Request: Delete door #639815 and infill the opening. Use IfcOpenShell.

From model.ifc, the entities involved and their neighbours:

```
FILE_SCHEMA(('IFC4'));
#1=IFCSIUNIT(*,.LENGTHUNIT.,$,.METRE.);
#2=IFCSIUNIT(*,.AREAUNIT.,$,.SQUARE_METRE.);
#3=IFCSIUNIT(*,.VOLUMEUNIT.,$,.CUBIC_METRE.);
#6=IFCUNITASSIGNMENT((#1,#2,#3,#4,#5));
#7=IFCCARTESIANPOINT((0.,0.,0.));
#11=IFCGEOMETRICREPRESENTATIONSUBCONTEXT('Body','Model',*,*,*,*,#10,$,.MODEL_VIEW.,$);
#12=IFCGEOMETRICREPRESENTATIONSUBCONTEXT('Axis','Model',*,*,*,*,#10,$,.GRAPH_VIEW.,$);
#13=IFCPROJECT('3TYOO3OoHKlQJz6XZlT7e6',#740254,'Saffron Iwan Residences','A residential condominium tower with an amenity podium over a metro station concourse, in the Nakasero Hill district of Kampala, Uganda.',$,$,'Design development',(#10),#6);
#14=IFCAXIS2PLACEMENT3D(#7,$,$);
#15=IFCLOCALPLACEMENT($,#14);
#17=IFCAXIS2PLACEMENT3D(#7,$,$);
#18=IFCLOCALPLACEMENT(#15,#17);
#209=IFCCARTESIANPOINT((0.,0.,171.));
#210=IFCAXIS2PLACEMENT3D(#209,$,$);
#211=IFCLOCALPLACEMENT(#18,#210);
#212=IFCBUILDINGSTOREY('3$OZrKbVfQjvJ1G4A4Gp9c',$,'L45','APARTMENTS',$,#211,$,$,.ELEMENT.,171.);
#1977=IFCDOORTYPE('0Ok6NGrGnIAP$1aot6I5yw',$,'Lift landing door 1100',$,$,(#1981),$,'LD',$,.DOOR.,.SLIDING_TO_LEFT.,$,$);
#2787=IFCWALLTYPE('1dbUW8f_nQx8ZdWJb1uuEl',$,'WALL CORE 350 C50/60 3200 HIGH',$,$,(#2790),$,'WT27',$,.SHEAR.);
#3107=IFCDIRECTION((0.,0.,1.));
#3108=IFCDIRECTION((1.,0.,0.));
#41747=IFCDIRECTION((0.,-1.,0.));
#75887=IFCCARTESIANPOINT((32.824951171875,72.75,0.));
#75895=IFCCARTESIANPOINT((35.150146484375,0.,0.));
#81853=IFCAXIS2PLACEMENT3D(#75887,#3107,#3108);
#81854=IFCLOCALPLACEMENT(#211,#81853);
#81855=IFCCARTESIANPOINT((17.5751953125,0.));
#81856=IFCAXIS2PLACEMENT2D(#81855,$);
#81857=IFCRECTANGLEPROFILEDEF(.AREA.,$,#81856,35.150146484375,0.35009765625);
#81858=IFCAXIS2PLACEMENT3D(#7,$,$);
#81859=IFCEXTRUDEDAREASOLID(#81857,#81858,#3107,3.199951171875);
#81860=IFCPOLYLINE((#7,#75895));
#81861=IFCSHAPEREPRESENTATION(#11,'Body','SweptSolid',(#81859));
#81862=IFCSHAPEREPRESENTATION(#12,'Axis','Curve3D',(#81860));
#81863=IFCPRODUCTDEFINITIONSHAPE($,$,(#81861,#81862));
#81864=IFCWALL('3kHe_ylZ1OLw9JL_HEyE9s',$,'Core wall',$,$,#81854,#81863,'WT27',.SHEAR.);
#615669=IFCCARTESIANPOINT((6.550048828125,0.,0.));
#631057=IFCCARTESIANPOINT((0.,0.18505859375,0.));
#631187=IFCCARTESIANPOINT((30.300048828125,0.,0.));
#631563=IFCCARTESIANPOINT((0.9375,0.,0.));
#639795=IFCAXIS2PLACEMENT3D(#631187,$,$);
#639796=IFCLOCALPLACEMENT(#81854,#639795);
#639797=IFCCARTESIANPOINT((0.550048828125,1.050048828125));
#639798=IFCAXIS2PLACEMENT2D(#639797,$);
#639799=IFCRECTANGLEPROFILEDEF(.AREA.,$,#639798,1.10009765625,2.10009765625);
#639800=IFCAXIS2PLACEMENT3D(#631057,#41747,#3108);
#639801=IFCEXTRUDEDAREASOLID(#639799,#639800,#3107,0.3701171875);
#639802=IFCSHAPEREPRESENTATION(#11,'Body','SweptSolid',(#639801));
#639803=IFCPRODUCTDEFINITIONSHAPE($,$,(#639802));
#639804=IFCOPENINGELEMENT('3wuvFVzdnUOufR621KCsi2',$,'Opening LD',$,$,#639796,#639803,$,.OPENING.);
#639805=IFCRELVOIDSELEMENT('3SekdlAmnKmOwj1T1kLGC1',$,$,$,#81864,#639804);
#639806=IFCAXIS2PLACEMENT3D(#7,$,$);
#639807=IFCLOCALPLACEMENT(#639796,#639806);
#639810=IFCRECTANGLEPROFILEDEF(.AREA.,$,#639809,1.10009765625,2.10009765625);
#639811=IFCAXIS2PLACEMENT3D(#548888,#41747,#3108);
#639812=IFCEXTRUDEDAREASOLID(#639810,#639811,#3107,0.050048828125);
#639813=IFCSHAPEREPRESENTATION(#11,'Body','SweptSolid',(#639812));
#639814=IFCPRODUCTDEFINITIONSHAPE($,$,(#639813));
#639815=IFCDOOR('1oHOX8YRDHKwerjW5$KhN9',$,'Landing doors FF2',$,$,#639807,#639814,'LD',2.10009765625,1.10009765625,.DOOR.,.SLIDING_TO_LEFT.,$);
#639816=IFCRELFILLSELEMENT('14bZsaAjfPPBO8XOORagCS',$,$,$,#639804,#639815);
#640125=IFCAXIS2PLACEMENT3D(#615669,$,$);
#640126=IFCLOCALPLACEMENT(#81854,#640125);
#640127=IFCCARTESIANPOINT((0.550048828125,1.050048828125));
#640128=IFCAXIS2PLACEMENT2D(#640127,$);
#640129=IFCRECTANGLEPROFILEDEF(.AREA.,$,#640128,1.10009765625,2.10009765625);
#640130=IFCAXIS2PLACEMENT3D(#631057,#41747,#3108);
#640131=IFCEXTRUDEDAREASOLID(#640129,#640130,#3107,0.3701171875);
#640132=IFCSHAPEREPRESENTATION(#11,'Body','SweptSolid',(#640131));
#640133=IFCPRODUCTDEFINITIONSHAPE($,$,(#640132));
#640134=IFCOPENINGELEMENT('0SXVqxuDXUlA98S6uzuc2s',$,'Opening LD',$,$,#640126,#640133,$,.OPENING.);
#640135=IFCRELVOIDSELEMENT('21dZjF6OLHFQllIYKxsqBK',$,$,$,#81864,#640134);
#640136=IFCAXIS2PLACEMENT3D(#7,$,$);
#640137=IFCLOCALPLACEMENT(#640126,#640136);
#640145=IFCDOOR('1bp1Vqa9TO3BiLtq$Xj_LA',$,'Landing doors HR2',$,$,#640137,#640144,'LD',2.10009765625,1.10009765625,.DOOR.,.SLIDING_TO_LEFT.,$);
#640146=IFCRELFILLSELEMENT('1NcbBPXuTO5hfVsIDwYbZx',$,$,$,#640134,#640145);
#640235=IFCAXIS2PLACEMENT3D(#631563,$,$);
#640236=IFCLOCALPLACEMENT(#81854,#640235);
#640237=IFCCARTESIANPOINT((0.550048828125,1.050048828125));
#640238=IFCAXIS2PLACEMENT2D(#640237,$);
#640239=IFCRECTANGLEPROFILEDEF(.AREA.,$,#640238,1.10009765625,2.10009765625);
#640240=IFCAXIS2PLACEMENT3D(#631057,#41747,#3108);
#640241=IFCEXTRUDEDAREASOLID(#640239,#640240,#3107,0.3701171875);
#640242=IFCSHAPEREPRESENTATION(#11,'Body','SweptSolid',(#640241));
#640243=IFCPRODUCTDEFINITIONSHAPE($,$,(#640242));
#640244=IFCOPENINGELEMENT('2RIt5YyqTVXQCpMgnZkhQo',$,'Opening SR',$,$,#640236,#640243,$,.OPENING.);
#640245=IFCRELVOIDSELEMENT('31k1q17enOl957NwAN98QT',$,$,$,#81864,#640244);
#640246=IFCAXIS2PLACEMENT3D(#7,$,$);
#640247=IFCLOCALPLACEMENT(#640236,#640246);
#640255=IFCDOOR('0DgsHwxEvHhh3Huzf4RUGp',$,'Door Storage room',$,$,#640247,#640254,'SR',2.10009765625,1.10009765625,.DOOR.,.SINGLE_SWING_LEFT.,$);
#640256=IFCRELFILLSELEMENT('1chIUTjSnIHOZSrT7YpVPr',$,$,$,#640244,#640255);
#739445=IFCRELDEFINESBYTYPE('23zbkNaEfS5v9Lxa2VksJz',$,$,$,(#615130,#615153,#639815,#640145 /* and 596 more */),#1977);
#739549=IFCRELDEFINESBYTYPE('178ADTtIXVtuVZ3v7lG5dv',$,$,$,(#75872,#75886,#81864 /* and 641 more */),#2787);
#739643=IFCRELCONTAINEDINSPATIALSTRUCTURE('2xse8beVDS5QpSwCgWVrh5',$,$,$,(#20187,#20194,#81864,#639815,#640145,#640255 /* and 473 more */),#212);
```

```python
import ifcopenshell
import ifcopenshell.api.feature
import ifcopenshell.api.root
import ifcopenshell.geom
import ifcopenshell.util.shape

model = ifcopenshell.open("model.ifc")
settings = ifcopenshell.geom.settings()


def volume(element):
    """Net volume in cubic metres, openings subtracted."""
    shape = ifcopenshell.geom.create_shape(settings, element)
    return ifcopenshell.util.shape.get_volume(shape.geometry)


door = model.by_guid("1oHOX8YRDHKwerjW5$KhN9")
opening = door.FillsVoids[0].RelatingOpeningElement
wall = opening.VoidsElements[0].RelatingBuildingElement
before = volume(wall)

ifcopenshell.api.root.remove_product(model, product=door)
ifcopenshell.api.feature.remove_feature(model, feature=opening)

after = volume(wall)

print(f"wall volume {before:.3f} -> {after:.3f} m3")

model.write("model_edited.ifc")
```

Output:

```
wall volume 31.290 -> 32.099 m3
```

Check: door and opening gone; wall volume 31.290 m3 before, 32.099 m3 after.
